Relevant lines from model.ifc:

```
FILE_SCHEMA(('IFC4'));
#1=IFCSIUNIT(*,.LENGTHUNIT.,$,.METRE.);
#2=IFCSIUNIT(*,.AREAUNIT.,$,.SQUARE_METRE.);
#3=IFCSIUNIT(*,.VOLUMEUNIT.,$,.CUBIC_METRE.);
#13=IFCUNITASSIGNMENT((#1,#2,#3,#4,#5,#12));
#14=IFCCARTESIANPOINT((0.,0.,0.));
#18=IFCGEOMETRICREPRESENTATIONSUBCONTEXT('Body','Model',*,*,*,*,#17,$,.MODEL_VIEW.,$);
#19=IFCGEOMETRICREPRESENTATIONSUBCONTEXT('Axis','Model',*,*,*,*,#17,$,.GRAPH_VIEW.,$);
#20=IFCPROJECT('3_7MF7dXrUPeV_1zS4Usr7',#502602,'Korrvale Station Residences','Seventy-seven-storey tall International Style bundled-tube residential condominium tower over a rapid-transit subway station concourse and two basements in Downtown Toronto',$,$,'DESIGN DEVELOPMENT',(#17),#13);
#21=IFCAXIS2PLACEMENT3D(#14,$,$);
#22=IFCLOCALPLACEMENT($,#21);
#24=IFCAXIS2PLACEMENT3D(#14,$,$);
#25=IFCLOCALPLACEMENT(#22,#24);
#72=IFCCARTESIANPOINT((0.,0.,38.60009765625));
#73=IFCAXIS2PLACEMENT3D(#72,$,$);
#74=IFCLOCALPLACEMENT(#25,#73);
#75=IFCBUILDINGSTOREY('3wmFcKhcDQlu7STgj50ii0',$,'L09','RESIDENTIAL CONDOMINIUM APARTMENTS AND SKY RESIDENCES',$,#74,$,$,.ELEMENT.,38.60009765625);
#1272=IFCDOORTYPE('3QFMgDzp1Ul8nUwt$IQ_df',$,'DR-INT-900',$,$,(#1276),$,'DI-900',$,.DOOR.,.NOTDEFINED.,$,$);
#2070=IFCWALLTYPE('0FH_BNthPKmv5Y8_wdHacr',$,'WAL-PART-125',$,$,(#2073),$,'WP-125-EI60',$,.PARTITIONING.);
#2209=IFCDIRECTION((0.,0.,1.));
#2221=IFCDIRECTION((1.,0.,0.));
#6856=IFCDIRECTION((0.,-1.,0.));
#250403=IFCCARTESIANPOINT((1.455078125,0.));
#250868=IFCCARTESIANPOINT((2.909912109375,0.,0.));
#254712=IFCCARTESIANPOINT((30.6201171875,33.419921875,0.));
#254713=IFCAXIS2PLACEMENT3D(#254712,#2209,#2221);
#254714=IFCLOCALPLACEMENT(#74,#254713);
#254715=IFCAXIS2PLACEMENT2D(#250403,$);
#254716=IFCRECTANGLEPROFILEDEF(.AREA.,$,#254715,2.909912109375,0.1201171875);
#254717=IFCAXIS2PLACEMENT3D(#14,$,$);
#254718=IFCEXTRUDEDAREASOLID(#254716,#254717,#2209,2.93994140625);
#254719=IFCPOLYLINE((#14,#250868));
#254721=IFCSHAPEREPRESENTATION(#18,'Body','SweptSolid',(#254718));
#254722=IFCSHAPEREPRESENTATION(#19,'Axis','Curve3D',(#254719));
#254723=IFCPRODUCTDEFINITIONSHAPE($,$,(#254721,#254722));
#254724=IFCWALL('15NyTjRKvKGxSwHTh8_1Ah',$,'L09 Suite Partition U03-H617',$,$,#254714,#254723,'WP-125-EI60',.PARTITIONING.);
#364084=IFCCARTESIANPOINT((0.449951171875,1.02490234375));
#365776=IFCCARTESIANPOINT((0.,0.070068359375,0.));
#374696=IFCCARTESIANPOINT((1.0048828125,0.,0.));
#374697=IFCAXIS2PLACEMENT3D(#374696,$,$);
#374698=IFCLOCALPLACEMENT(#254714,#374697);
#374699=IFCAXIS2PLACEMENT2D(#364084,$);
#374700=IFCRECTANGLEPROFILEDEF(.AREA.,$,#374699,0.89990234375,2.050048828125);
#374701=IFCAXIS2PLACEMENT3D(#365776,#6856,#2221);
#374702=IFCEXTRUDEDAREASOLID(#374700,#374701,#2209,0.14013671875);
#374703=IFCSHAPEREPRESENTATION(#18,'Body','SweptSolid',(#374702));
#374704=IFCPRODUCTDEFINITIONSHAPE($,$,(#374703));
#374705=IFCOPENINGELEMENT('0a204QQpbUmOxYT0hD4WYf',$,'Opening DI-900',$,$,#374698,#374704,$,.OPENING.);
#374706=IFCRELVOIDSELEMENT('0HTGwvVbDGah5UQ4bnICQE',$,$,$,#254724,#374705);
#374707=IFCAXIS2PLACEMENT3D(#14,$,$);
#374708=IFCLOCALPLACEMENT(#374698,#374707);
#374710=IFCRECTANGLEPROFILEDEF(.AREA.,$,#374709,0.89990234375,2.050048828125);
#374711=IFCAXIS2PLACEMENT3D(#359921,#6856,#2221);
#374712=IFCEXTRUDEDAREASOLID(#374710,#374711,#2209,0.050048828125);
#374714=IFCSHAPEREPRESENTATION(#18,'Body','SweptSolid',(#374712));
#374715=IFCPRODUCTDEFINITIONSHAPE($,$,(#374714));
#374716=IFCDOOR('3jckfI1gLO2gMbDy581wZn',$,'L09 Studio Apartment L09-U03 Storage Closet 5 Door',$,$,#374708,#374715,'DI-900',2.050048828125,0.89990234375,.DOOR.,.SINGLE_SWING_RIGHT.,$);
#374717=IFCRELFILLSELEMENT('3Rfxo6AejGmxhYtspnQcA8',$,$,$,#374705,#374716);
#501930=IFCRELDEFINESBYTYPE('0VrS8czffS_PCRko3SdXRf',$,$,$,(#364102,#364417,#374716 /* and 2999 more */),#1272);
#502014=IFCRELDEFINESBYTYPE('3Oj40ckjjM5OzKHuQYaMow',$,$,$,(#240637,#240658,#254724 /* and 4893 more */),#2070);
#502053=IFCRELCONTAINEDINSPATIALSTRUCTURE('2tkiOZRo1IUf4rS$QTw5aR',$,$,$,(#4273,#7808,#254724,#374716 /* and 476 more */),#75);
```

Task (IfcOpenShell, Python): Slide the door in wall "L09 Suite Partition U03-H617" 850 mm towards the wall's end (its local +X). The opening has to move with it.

```python
import ifcopenshell
import ifcopenshell.api.geometry
import ifcopenshell.util.placement

model = ifcopenshell.open("model.ifc")

door = model.by_guid("3jckfI1gLO2gMbDy581wZn")
opening = door.FillsVoids[0].RelatingOpeningElement
wall = opening.VoidsElements[0].RelatingBuildingElement

wall_matrix = ifcopenshell.util.placement.get_local_placement(wall.ObjectPlacement)
shift = wall_matrix[:3, 0] * 0.85
before = ifcopenshell.util.placement.get_local_placement(door.ObjectPlacement)[:3, 3].copy()

# The door is placed relative to its opening, so it follows when the opening moves.
matrix = ifcopenshell.util.placement.get_local_placement(opening.ObjectPlacement)
matrix[:3, 3] += shift
ifcopenshell.api.geometry.edit_object_placement(
    model, product=opening, matrix=matrix, is_si=False, should_transform_children=True
)

after = ifcopenshell.util.placement.get_local_placement(door.ObjectPlacement)[:3, 3]
print("door moved by", (after - before).round(3) + 0.0)

model.write("model-out.ifc")
```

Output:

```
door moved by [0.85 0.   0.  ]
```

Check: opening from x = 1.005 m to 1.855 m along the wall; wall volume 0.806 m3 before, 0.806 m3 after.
